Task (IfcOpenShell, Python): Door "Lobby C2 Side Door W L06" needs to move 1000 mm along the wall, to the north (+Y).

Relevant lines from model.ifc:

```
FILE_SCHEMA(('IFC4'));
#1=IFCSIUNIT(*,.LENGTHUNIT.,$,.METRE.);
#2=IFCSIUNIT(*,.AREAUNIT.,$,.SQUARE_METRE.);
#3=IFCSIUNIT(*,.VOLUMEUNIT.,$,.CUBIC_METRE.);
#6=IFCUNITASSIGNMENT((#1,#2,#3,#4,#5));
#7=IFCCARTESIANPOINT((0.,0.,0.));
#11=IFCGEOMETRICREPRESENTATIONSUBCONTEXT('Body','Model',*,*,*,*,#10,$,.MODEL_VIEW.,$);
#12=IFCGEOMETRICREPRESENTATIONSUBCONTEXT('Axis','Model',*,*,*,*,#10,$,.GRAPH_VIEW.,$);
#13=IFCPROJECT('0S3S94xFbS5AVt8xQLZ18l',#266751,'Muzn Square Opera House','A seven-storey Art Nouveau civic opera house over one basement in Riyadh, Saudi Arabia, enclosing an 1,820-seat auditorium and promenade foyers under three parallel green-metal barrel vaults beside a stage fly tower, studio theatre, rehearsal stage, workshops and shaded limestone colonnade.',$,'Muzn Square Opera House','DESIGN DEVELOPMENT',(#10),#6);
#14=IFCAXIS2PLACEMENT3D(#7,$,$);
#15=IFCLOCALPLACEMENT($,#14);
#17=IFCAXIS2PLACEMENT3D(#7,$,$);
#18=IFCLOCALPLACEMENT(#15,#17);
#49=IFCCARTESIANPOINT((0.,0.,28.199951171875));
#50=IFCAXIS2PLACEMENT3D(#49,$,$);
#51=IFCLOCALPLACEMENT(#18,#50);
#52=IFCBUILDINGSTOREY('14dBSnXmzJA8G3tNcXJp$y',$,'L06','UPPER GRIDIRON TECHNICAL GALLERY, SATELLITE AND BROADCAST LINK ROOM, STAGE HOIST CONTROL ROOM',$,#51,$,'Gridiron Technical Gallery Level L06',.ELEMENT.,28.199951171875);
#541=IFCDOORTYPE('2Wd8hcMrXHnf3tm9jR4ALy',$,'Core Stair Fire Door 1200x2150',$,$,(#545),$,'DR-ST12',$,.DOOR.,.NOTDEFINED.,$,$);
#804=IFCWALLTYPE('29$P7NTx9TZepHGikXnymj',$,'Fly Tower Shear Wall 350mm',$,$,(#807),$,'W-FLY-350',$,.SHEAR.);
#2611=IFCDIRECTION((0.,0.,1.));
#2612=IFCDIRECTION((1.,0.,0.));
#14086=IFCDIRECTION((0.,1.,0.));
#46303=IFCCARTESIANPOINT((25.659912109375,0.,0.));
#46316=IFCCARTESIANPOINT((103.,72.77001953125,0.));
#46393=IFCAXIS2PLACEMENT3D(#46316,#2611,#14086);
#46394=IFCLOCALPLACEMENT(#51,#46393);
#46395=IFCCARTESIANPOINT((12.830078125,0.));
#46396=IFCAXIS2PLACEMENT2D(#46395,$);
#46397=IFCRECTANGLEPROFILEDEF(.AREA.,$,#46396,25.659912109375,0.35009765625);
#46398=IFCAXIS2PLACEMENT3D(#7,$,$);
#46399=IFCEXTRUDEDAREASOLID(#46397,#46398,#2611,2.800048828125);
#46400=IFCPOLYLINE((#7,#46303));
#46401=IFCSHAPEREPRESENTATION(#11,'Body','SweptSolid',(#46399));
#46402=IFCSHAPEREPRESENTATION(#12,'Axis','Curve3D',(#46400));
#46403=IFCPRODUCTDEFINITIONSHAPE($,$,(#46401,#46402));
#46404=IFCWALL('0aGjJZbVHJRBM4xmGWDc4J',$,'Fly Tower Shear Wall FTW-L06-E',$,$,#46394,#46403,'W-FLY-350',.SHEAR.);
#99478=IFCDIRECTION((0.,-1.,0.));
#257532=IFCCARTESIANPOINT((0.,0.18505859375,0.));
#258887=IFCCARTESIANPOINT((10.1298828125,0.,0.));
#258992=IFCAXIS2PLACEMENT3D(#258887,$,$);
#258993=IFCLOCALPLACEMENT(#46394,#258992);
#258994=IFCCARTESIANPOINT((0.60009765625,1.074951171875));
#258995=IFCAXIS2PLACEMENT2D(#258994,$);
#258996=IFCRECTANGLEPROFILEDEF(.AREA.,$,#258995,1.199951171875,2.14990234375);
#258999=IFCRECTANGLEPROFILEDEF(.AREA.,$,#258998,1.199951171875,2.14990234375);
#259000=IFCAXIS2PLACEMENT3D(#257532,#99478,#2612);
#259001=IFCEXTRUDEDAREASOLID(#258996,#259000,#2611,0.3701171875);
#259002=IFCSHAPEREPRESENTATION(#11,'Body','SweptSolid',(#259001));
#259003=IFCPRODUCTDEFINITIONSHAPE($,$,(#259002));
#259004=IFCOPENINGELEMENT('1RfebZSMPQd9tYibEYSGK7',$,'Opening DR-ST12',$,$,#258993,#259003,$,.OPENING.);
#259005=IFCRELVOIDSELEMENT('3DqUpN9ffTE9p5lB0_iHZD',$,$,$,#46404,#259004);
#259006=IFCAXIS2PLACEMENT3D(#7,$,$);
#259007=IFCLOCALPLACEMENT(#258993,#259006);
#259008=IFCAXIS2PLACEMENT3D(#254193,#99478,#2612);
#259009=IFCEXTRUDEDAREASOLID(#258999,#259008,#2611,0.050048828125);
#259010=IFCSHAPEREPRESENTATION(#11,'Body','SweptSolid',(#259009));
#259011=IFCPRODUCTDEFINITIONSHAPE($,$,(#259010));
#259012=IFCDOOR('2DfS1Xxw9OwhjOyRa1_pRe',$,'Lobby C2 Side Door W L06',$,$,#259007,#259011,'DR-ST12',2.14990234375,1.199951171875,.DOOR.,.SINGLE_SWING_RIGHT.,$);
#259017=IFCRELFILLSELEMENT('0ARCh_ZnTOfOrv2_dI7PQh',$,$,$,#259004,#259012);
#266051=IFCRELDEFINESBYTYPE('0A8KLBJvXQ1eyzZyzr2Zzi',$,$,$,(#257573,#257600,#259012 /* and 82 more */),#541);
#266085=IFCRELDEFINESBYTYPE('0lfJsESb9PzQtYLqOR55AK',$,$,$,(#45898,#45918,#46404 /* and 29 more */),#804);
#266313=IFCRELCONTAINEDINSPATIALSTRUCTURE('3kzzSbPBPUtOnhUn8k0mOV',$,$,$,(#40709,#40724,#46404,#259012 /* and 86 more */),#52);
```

```python
import ifcopenshell
import ifcopenshell.api.geometry
import ifcopenshell.util.placement

model = ifcopenshell.open("model.ifc")

door = model.by_guid("2DfS1Xxw9OwhjOyRa1_pRe")
opening = door.FillsVoids[0].RelatingOpeningElement
wall = opening.VoidsElements[0].RelatingBuildingElement

wall_matrix = ifcopenshell.util.placement.get_local_placement(wall.ObjectPlacement)
shift = wall_matrix[:3, 0] * 1.0
before = ifcopenshell.util.placement.get_local_placement(door.ObjectPlacement)[:3, 3].copy()

# The door is placed relative to its opening, so it follows when the opening moves.
matrix = ifcopenshell.util.placement.get_local_placement(opening.ObjectPlacement)
matrix[:3, 3] += shift
ifcopenshell.api.geometry.edit_object_placement(
    model, product=opening, matrix=matrix, is_si=False, should_transform_children=True
)

after = ifcopenshell.util.placement.get_local_placement(door.ObjectPlacement)[:3, 3]
print("door moved by", (after - before).round(3) + 0.0)

model.write("model_edited.ifc")
```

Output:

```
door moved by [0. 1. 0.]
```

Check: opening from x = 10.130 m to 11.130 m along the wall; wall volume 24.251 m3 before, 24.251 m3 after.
